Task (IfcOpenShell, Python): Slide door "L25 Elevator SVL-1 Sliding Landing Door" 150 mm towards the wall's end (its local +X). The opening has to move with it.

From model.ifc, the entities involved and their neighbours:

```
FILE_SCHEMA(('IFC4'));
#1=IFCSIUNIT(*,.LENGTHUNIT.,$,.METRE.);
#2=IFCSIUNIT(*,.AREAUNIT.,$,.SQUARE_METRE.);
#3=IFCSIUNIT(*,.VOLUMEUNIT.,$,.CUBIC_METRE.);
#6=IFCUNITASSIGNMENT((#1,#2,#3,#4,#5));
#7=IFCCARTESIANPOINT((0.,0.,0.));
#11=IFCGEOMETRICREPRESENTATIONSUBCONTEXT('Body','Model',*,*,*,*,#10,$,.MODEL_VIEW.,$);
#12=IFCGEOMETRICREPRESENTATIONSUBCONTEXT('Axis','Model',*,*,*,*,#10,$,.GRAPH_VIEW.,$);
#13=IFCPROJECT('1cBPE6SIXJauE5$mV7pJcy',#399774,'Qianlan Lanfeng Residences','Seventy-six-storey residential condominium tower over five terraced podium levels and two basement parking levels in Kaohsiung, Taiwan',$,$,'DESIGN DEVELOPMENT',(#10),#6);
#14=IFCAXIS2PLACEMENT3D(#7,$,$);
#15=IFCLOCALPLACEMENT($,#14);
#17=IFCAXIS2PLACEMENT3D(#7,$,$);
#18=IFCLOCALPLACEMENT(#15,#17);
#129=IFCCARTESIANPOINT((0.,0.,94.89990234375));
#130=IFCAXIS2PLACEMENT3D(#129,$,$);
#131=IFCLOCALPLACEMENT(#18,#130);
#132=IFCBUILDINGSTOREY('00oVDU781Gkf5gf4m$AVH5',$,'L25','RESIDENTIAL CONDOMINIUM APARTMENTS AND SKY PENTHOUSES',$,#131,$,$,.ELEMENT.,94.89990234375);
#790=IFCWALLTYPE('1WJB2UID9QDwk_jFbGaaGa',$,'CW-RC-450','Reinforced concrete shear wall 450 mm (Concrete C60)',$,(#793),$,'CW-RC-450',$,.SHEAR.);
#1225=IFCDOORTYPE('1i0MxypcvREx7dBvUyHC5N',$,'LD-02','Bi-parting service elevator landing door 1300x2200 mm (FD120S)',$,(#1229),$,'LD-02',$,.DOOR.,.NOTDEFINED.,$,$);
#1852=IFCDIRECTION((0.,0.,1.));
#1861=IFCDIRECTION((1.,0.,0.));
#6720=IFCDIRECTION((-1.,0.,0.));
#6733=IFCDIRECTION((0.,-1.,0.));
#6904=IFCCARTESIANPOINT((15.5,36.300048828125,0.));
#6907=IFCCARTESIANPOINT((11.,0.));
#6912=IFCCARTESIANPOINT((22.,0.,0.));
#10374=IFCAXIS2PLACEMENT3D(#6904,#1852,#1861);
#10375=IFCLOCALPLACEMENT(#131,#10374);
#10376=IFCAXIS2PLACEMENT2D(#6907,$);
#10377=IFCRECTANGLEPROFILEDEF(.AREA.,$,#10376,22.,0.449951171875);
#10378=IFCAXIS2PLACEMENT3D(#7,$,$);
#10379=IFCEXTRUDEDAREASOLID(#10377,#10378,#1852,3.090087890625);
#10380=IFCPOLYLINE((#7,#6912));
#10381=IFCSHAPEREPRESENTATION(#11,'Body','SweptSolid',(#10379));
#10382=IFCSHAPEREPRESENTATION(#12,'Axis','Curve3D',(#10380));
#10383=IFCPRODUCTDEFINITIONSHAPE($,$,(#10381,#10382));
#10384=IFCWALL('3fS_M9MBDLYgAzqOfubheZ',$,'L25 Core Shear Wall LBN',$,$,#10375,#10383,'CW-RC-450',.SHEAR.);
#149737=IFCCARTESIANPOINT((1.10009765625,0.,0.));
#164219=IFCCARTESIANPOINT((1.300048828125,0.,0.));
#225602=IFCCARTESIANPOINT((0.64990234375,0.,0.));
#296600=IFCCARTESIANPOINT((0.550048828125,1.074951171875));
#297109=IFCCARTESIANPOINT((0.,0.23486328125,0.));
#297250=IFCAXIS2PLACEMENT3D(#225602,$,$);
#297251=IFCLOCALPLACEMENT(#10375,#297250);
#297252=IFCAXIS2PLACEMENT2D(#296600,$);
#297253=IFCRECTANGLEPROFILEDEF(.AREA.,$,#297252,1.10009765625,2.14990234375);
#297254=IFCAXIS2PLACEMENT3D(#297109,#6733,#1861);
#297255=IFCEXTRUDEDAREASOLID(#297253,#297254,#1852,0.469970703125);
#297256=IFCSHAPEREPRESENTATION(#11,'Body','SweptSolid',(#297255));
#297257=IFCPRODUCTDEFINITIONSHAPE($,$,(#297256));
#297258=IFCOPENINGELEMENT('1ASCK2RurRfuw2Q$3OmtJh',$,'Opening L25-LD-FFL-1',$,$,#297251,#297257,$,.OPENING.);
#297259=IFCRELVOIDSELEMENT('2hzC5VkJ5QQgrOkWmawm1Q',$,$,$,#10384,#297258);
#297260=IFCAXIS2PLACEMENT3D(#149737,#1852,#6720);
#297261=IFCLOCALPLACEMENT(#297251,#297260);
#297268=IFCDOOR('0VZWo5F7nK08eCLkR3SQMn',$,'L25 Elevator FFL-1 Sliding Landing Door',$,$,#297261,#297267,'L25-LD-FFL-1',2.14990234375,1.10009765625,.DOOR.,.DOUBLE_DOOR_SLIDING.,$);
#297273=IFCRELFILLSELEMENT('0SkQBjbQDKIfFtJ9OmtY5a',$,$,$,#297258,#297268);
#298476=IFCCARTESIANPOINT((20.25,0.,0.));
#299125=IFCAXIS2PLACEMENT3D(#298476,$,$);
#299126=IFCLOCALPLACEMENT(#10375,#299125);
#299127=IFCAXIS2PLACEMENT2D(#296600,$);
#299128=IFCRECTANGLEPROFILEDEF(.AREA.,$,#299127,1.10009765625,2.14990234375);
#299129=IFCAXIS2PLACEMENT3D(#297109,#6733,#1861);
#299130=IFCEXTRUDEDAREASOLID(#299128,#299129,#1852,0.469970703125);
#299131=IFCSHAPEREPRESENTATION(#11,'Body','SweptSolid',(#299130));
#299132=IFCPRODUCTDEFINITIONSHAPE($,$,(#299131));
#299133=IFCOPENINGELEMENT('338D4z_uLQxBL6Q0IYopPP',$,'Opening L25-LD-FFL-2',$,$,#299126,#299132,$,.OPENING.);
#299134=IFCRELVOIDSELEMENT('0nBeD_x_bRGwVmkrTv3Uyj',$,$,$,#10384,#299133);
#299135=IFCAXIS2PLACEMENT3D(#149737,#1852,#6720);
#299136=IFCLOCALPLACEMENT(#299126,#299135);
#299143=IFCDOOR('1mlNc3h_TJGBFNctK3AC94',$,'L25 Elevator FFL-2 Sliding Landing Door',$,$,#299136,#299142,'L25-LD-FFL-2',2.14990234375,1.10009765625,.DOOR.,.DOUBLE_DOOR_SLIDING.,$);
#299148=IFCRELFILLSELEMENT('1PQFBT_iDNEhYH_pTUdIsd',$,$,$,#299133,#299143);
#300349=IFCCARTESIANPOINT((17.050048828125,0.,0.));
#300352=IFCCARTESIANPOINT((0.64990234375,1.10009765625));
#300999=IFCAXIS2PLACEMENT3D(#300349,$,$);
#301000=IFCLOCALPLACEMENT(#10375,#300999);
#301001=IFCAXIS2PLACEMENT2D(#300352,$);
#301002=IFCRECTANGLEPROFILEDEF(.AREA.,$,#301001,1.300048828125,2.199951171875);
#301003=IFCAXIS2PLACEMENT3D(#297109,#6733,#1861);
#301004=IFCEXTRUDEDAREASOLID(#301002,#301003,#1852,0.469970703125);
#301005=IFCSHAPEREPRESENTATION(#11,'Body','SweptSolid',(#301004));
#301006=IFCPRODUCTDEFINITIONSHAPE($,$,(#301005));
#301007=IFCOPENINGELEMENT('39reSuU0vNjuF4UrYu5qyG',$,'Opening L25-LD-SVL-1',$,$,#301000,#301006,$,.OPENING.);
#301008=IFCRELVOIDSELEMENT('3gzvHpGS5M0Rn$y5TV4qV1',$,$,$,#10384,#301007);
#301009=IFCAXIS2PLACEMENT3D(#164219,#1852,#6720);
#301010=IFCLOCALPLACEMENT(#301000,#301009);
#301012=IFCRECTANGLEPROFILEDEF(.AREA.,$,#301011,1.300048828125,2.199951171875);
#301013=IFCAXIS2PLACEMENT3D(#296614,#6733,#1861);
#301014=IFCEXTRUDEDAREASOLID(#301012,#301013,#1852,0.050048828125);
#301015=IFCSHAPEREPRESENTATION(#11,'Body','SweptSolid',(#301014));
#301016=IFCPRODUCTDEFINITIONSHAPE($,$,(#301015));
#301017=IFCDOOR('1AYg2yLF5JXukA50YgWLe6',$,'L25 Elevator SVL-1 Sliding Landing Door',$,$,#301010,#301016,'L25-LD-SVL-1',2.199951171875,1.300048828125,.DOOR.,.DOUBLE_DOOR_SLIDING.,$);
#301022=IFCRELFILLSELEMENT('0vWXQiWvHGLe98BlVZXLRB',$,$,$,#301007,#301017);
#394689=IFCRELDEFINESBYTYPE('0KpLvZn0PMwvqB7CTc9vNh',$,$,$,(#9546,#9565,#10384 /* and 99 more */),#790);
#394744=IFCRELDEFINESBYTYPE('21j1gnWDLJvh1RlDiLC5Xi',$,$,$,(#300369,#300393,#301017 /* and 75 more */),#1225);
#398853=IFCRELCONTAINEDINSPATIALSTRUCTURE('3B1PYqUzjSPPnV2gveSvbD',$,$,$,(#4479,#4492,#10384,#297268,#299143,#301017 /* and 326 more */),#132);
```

```python
import ifcopenshell
import ifcopenshell.api.geometry
import ifcopenshell.util.placement

model = ifcopenshell.open("model.ifc")

door = model.by_guid("1AYg2yLF5JXukA50YgWLe6")
opening = door.FillsVoids[0].RelatingOpeningElement
wall = opening.VoidsElements[0].RelatingBuildingElement

wall_matrix = ifcopenshell.util.placement.get_local_placement(wall.ObjectPlacement)
shift = wall_matrix[:3, 0] * 0.15
before = ifcopenshell.util.placement.get_local_placement(door.ObjectPlacement)[:3, 3].copy()

# The door is placed relative to its opening, so it follows when the opening moves.
matrix = ifcopenshell.util.placement.get_local_placement(opening.ObjectPlacement)
matrix[:3, 3] += shift
ifcopenshell.api.geometry.edit_object_placement(
    model, product=opening, matrix=matrix, is_si=False, should_transform_children=True
)

after = ifcopenshell.util.placement.get_local_placement(door.ObjectPlacement)[:3, 3]
print("door moved by", (after - before).round(3) + 0.0)

model.write("model-out.ifc")
```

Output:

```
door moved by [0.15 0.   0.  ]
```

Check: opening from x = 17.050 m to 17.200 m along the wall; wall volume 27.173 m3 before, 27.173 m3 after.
